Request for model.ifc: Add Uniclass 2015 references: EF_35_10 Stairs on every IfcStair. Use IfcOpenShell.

First a look at what the model holds.

```python
import ifcopenshell

model = ifcopenshell.open("model.ifc")
print(model.schema)
print("classifications:", [c.Name for c in model.by_type("IfcClassification")])
for ifc_class in ("IfcDoor", "IfcRoof", "IfcStair", "IfcWall", "IfcWindow"):
    print(ifc_class, len(model.by_type(ifc_class)))
```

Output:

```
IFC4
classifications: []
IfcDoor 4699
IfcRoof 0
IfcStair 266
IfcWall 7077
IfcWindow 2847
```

```python
import ifcopenshell
import ifcopenshell.api.classification

model = ifcopenshell.open("model.ifc")

system = ifcopenshell.api.classification.add_classification(model, classification="Uniclass 2015")

codes = {
    "IfcStair": ("EF_35_10", "Stairs"),
}
for ifc_class, (code, name) in codes.items():
    products = model.by_type(ifc_class)
    ifcopenshell.api.classification.add_reference(
        model, products=products, classification=system, identification=code, name=name
    )
    print(code, len(products))

model.write("model-out.ifc")
```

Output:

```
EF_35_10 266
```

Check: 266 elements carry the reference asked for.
